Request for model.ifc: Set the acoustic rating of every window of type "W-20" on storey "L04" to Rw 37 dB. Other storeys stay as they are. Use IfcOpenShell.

First a look at what the model holds.

```python
import ifcopenshell
import ifcopenshell.util.element

model = ifcopenshell.open("model.ifc")
print(model.schema)
storey = next(s for s in model.by_type("IfcBuildingStorey") if s.Name == "L04")
windows = [e for e in ifcopenshell.util.element.get_decomposition(storey) if e.is_a("IfcWindow")]
seen = {}
for e in windows:
    element_type = ifcopenshell.util.element.get_type(e)
    key = (element_type.Name if element_type != e and element_type else None, ifcopenshell.util.element.get_pset(e, "Pset_WindowCommon", "AcousticRating"))
    seen[key] = seen.get(key, 0) + 1
for (name, value), count in sorted(seen.items(), key=str):
    print(count, "x", name, "|", value)
```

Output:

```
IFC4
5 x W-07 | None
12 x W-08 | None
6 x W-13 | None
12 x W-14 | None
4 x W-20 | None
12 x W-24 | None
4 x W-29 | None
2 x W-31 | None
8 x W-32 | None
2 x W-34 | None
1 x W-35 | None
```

```python
import ifcopenshell
import ifcopenshell.api.pset
import ifcopenshell.util.element

model = ifcopenshell.open("model.ifc")

storey = next(s for s in model.by_type("IfcBuildingStorey") if s.Name == "L04")
windows = [e for e in ifcopenshell.util.element.get_decomposition(storey) if e.is_a("IfcWindow")]

count = 0
for e in windows:
    element_type = ifcopenshell.util.element.get_type(e)
    if element_type in (None, e) or element_type.Name != "W-20":
        continue
    # add_pset returns the element's existing set when there is one.
    pset = ifcopenshell.api.pset.add_pset(model, product=e, name="Pset_WindowCommon")
    ifcopenshell.api.pset.edit_pset(model, pset=pset, properties={"AcousticRating": "Rw 37 dB"})
    count += 1

print(count, "windows updated")

model.write("model_rev.ifc")
```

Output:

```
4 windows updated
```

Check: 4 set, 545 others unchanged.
